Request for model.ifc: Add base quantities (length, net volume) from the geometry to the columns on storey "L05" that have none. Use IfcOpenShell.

First a look at what the model holds.

```python
import ifcopenshell
import ifcopenshell.util.element
import ifcopenshell.util.unit

model = ifcopenshell.open("model.ifc")
print(model.schema)
for unit_type in ("LENGTHUNIT", "AREAUNIT", "VOLUMEUNIT"):
    print(unit_type, ifcopenshell.util.unit.calculate_unit_scale(model, unit_type))
storey = next(s for s in model.by_type("IfcBuildingStorey") if s.Name == "L05")
columns = [e for e in ifcopenshell.util.element.get_decomposition(storey) if e.is_a("IfcColumn")]
for e in sorted(columns, key=lambda e: e.id()):
    print(e.id(), e.is_a(), e.Name, list(ifcopenshell.util.element.get_psets(e, qtos_only=True)), sep=" | ")
```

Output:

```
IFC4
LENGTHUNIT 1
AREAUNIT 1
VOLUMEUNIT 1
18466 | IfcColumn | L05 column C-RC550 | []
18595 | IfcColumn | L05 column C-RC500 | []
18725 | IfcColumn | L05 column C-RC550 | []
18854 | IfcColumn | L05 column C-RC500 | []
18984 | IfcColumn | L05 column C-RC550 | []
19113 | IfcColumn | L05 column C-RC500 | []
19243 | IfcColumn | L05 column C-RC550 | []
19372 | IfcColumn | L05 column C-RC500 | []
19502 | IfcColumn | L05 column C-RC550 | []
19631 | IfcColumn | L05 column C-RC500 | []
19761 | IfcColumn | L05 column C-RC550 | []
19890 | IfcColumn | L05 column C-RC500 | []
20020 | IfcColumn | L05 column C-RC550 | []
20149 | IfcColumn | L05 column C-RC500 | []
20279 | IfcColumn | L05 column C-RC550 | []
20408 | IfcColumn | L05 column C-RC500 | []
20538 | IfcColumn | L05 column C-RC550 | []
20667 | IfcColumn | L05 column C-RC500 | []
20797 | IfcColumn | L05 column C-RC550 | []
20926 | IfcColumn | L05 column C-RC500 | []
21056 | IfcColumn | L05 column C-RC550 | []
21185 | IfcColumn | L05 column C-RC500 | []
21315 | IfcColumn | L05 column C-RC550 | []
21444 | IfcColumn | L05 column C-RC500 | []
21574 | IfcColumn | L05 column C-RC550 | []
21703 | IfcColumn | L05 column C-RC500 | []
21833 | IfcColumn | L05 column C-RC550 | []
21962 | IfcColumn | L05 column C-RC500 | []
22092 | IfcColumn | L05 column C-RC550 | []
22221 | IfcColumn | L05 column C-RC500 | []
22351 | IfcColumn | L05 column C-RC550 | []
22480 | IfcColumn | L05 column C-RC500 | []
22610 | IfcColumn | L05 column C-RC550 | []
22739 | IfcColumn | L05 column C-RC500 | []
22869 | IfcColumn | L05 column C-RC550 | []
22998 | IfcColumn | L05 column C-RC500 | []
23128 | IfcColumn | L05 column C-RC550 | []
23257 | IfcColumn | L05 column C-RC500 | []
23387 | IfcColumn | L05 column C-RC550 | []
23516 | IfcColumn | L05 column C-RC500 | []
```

```python
import ifcopenshell
import ifcopenshell.api.pset
import ifcopenshell.geom
import ifcopenshell.util.element
import ifcopenshell.util.shape
import ifcopenshell.util.unit

model = ifcopenshell.open("model.ifc")
unit_scale = ifcopenshell.util.unit.calculate_unit_scale(model)
volume_scale = ifcopenshell.util.unit.calculate_unit_scale(model, "VOLUMEUNIT")
settings = ifcopenshell.geom.settings()

storey = next(s for s in model.by_type("IfcBuildingStorey") if s.Name == "L05")
columns = [e for e in ifcopenshell.util.element.get_decomposition(storey) if e.is_a("IfcColumn")]

for e in sorted(columns, key=lambda e: e.id()):
    if ifcopenshell.util.element.get_psets(e, qtos_only=True, should_inherit=False):
        continue
    # Geometry comes back in metres, in the element's own axes.
    shape = ifcopenshell.geom.create_shape(settings, e)
    values = {
        "Length": ifcopenshell.util.shape.get_z(shape.geometry) / unit_scale,
        "NetVolume": ifcopenshell.util.shape.get_volume(shape.geometry) / volume_scale,
    }
    qto = ifcopenshell.api.pset.add_qto(model, product=e, name="Qto_ColumnBaseQuantities")
    ifcopenshell.api.pset.edit_qto(model, qto=qto, properties=values)
    print(e.id(), {k: round(v, 3) for k, v in values.items()})

model.write("model-out.ifc")
```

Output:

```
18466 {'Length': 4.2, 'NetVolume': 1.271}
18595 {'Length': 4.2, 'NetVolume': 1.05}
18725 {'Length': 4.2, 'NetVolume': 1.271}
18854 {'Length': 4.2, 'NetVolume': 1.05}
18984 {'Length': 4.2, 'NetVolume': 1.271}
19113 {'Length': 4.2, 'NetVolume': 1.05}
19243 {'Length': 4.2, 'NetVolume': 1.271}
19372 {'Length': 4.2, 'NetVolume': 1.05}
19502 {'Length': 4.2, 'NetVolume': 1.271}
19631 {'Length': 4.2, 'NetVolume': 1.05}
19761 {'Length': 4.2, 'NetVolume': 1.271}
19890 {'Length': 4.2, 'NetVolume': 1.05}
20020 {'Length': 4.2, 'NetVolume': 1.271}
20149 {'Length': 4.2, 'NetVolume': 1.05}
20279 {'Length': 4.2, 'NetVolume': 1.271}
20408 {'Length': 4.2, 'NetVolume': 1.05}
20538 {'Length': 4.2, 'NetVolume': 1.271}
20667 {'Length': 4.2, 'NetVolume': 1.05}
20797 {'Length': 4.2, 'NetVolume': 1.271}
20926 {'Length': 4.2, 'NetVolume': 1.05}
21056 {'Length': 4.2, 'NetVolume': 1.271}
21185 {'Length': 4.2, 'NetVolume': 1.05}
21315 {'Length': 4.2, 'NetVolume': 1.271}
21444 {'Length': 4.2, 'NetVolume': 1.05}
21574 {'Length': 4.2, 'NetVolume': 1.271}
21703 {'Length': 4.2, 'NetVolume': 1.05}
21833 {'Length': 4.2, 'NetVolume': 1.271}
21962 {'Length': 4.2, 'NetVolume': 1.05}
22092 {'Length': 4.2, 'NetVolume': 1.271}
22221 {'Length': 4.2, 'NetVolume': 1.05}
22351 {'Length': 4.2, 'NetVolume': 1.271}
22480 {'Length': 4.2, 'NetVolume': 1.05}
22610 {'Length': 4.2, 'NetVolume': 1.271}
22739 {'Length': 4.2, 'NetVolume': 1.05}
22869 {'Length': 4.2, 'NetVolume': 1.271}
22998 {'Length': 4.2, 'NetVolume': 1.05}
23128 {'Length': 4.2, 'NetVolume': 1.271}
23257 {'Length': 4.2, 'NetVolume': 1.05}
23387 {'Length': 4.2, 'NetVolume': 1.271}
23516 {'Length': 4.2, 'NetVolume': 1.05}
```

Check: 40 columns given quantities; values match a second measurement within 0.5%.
